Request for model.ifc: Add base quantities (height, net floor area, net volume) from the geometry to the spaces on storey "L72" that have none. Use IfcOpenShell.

First a look at what the model holds.

```python
import ifcopenshell
import ifcopenshell.util.element
import ifcopenshell.util.unit

model = ifcopenshell.open("model.ifc")
print(model.schema)
for unit_type in ("LENGTHUNIT", "AREAUNIT", "VOLUMEUNIT"):
    print(unit_type, ifcopenshell.util.unit.calculate_unit_scale(model, unit_type))
storey = next(s for s in model.by_type("IfcBuildingStorey") if s.Name == "L72")
spaces = [e for e in ifcopenshell.util.element.get_decomposition(storey) if e.is_a("IfcSpace")]
for e in sorted(spaces, key=lambda e: e.id()):
    print(e.id(), e.is_a(), e.Name, list(ifcopenshell.util.element.get_psets(e, qtos_only=True)), sep=" | ")
```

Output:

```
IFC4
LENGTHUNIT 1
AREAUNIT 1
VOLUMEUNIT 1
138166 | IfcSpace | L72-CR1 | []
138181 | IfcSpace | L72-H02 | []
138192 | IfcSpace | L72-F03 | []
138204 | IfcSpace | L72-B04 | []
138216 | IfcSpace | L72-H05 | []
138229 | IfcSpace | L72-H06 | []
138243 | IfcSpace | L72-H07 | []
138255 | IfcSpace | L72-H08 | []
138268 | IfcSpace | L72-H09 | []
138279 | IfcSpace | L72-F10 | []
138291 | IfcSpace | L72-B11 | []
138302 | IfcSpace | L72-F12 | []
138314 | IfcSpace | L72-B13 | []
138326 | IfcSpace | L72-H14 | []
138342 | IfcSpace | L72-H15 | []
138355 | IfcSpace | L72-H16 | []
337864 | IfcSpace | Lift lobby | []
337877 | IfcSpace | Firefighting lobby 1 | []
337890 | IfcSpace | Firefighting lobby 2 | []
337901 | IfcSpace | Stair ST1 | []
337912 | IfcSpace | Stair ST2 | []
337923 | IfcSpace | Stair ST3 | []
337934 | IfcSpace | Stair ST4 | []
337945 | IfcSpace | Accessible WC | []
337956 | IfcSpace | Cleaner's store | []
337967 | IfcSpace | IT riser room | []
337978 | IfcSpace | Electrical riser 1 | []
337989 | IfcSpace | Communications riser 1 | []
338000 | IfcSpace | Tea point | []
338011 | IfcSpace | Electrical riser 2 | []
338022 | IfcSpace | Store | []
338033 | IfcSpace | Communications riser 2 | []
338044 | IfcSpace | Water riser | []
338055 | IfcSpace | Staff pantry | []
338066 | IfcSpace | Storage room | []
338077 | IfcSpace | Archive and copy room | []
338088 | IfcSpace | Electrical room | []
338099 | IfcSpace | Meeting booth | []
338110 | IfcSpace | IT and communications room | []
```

```python
import ifcopenshell
import ifcopenshell.api.pset
import ifcopenshell.geom
import ifcopenshell.util.element
import ifcopenshell.util.shape
import ifcopenshell.util.unit

model = ifcopenshell.open("model.ifc")
unit_scale = ifcopenshell.util.unit.calculate_unit_scale(model)
area_scale = ifcopenshell.util.unit.calculate_unit_scale(model, "AREAUNIT")
volume_scale = ifcopenshell.util.unit.calculate_unit_scale(model, "VOLUMEUNIT")
settings = ifcopenshell.geom.settings()

storey = next(s for s in model.by_type("IfcBuildingStorey") if s.Name == "L72")
spaces = [e for e in ifcopenshell.util.element.get_decomposition(storey) if e.is_a("IfcSpace")]

for e in sorted(spaces, key=lambda e: e.id()):
    if ifcopenshell.util.element.get_psets(e, qtos_only=True, should_inherit=False):
        continue
    # Geometry comes back in metres, in the element's own axes.
    shape = ifcopenshell.geom.create_shape(settings, e)
    values = {
        "Height": ifcopenshell.util.shape.get_z(shape.geometry) / unit_scale,
        "NetFloorArea": ifcopenshell.util.shape.get_footprint_area(shape.geometry) / area_scale,
        "NetVolume": ifcopenshell.util.shape.get_volume(shape.geometry) / volume_scale,
    }
    qto = ifcopenshell.api.pset.add_qto(model, product=e, name="Qto_SpaceBaseQuantities")
    ifcopenshell.api.pset.edit_qto(model, qto=qto, properties=values)
    print(e.id(), {k: round(v, 3) for k, v in values.items()})

model.write("model_updated.ifc")
```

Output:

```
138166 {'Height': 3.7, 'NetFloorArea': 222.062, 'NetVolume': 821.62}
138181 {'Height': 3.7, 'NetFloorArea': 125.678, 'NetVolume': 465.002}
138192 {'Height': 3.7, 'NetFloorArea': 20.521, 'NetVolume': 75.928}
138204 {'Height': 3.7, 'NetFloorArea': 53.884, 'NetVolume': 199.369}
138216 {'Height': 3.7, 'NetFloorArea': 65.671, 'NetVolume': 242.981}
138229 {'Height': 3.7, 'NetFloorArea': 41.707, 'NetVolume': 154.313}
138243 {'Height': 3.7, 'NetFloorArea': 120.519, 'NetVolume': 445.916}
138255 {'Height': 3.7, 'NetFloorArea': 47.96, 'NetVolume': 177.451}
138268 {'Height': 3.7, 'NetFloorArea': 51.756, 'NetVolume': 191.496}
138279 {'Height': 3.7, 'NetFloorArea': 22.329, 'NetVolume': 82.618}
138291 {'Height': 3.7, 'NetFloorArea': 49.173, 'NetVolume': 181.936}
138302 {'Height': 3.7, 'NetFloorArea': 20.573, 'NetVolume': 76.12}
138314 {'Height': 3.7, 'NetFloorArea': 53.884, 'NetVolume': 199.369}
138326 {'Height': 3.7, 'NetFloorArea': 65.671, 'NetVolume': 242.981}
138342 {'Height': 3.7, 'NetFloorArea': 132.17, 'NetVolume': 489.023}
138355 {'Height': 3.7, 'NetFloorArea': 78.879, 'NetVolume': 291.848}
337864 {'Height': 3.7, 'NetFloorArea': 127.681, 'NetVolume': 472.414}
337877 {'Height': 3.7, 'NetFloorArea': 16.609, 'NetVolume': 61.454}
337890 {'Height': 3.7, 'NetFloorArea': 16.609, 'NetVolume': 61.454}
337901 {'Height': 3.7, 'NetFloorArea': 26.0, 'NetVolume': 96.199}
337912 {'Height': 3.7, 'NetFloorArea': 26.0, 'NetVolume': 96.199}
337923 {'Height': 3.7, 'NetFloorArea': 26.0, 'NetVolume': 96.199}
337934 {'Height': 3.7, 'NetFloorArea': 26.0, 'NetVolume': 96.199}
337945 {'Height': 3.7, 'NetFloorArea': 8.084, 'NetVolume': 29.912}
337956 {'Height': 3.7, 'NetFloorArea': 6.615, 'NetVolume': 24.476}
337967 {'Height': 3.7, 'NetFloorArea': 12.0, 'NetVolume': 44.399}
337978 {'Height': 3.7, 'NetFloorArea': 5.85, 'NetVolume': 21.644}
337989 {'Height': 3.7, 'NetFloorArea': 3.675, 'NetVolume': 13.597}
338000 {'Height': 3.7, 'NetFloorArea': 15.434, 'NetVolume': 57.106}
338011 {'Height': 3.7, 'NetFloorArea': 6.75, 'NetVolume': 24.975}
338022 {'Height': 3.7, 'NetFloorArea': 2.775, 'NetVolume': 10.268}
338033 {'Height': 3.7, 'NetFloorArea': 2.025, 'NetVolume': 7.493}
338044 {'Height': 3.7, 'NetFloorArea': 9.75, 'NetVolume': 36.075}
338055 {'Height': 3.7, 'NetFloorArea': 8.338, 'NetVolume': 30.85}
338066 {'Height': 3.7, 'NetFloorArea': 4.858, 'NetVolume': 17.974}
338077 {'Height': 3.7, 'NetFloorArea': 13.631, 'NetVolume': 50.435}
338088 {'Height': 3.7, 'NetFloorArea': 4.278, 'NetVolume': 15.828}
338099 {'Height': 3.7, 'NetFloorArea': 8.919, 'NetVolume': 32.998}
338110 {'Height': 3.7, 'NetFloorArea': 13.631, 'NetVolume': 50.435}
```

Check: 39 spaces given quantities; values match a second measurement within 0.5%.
